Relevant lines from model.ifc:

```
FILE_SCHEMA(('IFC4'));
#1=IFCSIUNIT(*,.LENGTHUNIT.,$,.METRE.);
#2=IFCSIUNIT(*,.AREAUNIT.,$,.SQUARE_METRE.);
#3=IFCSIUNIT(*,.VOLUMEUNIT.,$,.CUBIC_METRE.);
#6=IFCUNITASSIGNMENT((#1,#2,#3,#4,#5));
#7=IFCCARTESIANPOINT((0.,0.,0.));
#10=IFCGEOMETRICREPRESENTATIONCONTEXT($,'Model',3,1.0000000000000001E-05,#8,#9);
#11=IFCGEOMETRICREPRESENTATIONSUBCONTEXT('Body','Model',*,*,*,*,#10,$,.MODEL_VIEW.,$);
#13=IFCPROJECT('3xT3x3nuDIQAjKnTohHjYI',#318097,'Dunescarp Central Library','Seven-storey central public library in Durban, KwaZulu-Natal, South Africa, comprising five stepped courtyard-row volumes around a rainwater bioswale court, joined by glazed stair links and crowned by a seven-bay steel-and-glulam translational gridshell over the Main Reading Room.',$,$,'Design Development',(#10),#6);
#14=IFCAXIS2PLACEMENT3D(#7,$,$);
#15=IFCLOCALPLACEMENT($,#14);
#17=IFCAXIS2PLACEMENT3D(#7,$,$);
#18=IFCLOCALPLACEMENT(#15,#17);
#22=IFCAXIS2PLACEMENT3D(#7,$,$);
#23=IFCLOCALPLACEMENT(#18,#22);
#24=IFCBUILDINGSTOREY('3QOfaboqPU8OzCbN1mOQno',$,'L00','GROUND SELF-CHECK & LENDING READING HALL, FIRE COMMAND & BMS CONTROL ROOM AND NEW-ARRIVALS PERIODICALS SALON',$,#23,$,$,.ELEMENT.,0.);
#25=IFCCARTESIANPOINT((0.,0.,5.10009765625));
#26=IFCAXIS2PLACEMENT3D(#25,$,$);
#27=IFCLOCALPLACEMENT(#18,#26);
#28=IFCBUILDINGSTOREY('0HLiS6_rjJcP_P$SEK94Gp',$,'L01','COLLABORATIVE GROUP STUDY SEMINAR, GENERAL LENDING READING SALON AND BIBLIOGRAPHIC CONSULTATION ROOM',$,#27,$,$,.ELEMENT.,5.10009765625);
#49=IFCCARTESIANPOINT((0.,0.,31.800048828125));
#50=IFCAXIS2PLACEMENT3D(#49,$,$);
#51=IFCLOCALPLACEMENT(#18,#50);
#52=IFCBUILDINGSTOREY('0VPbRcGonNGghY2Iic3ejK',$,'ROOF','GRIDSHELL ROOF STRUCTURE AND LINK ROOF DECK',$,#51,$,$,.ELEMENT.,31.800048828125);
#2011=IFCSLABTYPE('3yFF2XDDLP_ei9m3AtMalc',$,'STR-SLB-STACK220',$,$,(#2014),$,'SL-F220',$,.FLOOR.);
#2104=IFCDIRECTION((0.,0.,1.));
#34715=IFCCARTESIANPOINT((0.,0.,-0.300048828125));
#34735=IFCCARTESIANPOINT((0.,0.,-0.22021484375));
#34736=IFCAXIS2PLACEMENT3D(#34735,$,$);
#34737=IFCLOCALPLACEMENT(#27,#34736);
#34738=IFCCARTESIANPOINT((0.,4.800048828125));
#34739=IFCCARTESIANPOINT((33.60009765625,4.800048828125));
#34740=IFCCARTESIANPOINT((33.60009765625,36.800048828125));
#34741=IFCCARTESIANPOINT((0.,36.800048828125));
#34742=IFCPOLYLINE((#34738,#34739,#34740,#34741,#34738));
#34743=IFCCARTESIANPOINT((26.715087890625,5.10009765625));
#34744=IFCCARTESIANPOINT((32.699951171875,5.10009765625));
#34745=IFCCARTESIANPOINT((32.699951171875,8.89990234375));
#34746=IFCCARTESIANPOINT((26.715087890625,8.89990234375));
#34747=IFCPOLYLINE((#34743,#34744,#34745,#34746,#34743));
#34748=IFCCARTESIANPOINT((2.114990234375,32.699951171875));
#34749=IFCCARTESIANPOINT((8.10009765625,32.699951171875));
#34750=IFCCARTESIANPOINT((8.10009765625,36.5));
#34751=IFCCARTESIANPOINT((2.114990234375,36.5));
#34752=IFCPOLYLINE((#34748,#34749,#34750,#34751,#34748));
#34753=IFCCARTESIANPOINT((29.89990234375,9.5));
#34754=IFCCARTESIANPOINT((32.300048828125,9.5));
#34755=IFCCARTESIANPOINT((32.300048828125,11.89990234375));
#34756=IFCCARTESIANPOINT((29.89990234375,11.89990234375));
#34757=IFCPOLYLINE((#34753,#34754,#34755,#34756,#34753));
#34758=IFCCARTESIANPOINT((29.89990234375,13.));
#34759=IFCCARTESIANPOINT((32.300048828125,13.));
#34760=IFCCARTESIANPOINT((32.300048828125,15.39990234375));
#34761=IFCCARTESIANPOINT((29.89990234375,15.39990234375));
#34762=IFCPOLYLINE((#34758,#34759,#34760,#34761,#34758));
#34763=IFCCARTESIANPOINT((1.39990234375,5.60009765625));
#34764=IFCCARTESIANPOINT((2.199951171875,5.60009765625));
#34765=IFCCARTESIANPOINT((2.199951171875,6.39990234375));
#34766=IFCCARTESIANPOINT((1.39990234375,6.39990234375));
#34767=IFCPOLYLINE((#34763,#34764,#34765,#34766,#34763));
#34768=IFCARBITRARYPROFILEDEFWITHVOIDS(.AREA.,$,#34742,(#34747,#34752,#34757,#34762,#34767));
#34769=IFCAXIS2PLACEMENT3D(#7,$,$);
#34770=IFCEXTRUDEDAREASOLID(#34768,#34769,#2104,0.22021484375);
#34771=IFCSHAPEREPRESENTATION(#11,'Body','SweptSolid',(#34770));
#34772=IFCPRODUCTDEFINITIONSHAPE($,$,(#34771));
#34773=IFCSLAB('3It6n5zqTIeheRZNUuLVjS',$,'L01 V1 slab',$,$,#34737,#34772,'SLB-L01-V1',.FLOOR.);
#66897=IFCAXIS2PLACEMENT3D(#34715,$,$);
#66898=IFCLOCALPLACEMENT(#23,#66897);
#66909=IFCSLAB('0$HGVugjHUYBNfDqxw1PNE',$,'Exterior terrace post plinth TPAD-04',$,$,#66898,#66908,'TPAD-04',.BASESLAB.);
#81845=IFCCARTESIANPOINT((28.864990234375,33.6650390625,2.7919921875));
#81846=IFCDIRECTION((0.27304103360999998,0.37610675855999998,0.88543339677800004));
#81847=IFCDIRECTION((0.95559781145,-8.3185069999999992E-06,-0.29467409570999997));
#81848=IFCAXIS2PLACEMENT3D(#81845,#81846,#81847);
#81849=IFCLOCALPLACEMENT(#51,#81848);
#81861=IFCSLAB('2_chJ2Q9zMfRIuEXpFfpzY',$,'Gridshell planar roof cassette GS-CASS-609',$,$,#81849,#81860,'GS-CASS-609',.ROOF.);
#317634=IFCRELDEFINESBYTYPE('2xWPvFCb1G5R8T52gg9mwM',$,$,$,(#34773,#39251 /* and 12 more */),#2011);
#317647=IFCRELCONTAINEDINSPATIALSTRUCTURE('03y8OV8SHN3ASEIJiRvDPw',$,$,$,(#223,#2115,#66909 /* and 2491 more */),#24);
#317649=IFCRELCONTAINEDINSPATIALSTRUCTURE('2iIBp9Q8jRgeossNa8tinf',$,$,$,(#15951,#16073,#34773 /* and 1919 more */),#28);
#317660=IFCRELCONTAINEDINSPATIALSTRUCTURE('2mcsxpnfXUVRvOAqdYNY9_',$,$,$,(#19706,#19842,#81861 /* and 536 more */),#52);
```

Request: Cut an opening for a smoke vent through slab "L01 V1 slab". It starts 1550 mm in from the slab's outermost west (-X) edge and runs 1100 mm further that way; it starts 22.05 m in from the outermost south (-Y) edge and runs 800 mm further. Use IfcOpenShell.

```python
import numpy as np
import ifcopenshell
import ifcopenshell.api.feature
import ifcopenshell.api.geometry
import ifcopenshell.api.root
import ifcopenshell.geom
import ifcopenshell.util.placement
import ifcopenshell.util.representation
import ifcopenshell.util.shape
import ifcopenshell.util.unit

model = ifcopenshell.open("model.ifc")
unit_scale = ifcopenshell.util.unit.calculate_unit_scale(model)
settings = ifcopenshell.geom.settings()


def volume(element):
    """Net volume in cubic metres, openings subtracted."""
    shape = ifcopenshell.geom.create_shape(settings, element)
    return ifcopenshell.util.shape.get_volume(shape.geometry)


slab = model.by_guid("3It6n5zqTIeheRZNUuLVjS")
before = volume(slab)

# Extent in the slab's own axes, in metres. The edges named are its -X and -Y sides.
slab_shape = ifcopenshell.geom.create_shape(settings, slab)
vertices = ifcopenshell.util.shape.get_vertices(slab_shape.geometry)
x_min, y_min, bottom = vertices.min(axis=0)
top = vertices[:, 2].max()

opening = ifcopenshell.api.root.create_entity(model, ifc_class="IfcOpeningElement", name="Smoke vent opening", predefined_type="OPENING")
context = ifcopenshell.util.representation.get_context(model, "Model", "Body", "MODEL_VIEW")
width, depth = 1.1, 0.8
outline = [(0.0, 0.0), (width, 0.0), (width, depth), (0.0, depth), (0.0, 0.0)]
# Overshoot both faces by 50 mm so the cut is clean.
shape = ifcopenshell.api.geometry.add_slab_representation(
    model, context=context, depth=top - bottom + 0.1, polyline=outline
)
ifcopenshell.api.geometry.assign_representation(model, product=opening, representation=shape)

matrix = ifcopenshell.util.placement.get_local_placement(slab.ObjectPlacement)
matrix[:, 3] = matrix @ np.append(np.array([x_min + 1.55, y_min + 22.05, bottom - 0.05]) / unit_scale, 1.0)
ifcopenshell.api.geometry.edit_object_placement(model, product=opening, matrix=matrix, is_si=False)
ifcopenshell.api.feature.add_feature(model, feature=opening, element=slab)

after = volume(slab)

print(f"slab volume {before:.3f} -> {after:.3f} m3")

model.write("model_updated.ifc")
```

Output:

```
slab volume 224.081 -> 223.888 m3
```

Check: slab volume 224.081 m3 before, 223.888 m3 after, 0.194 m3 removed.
